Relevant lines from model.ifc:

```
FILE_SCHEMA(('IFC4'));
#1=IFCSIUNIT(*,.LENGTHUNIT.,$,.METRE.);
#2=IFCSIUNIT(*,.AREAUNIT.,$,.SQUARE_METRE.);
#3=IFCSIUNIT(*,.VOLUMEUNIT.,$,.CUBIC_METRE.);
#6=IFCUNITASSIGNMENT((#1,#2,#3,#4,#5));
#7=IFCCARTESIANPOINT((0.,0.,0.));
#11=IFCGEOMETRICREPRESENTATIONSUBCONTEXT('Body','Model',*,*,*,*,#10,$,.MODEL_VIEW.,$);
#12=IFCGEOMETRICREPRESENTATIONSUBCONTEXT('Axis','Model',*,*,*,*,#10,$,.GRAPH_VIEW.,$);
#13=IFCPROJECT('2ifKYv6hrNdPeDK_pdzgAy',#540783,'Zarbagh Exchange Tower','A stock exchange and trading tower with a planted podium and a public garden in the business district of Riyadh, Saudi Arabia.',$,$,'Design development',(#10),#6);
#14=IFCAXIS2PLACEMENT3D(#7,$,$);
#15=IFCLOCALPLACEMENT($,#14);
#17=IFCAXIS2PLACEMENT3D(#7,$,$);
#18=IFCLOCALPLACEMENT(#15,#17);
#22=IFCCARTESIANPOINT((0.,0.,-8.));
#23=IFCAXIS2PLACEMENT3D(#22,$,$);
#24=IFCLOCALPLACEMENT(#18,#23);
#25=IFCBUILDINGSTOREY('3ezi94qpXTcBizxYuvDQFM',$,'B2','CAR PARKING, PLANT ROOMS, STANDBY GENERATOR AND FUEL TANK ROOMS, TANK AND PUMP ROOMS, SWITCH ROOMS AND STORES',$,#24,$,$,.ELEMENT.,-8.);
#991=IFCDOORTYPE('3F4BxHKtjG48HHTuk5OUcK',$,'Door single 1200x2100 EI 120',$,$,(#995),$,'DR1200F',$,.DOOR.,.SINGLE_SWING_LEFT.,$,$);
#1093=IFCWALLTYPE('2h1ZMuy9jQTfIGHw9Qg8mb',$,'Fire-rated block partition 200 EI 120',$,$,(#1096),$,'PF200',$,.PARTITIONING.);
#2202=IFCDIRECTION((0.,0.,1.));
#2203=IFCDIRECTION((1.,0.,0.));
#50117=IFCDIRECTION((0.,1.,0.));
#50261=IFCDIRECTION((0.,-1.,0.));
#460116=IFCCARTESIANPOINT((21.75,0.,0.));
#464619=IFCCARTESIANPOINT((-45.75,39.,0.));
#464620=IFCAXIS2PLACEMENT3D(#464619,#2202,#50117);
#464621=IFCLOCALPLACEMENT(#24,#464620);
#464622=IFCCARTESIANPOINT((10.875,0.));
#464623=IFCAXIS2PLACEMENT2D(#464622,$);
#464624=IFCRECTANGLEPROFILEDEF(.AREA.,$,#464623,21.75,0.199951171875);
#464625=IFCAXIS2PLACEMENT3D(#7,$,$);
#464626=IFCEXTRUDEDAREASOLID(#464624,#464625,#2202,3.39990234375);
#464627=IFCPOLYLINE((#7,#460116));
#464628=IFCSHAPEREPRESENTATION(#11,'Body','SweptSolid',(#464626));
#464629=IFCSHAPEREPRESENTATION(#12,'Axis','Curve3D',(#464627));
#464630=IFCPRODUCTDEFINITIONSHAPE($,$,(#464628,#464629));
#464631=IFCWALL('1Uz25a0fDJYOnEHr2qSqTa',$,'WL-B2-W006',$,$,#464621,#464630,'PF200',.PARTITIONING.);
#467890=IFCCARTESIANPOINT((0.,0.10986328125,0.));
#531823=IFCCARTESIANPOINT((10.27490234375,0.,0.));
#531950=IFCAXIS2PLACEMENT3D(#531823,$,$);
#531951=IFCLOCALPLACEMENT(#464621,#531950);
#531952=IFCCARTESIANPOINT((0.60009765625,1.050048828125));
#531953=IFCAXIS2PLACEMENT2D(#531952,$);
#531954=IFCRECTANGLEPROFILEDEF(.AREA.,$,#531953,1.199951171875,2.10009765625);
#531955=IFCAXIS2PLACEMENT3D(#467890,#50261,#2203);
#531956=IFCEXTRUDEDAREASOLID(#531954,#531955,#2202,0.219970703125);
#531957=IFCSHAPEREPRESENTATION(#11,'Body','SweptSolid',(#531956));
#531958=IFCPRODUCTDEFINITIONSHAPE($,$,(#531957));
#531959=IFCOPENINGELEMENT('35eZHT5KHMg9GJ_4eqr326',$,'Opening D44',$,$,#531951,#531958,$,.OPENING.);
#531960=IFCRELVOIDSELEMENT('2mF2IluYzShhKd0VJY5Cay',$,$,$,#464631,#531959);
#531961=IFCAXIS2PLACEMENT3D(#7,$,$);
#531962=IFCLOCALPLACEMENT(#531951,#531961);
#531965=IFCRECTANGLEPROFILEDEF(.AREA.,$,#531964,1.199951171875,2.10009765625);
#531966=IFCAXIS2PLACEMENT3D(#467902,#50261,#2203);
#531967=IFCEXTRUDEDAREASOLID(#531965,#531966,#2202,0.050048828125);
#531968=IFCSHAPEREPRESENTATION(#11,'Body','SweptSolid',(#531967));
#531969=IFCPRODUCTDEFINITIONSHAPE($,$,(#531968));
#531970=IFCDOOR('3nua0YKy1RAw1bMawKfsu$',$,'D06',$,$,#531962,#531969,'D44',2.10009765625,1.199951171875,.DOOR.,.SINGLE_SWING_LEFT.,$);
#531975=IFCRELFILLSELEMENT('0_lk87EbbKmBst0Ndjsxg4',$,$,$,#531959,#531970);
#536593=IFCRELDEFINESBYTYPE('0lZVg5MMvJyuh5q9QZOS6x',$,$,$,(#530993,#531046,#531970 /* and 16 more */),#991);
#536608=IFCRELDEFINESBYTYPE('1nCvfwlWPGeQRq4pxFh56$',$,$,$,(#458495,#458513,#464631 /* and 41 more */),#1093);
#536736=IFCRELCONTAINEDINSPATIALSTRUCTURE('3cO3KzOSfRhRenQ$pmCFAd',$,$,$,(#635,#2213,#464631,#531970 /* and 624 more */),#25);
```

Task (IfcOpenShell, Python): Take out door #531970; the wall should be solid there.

```python
import ifcopenshell
import ifcopenshell.api.feature
import ifcopenshell.api.root
import ifcopenshell.geom
import ifcopenshell.util.shape

model = ifcopenshell.open("model.ifc")
settings = ifcopenshell.geom.settings()


def volume(element):
    """Net volume in cubic metres, openings subtracted."""
    shape = ifcopenshell.geom.create_shape(settings, element)
    return ifcopenshell.util.shape.get_volume(shape.geometry)


door = model.by_guid("3nua0YKy1RAw1bMawKfsu$")
opening = door.FillsVoids[0].RelatingOpeningElement
wall = opening.VoidsElements[0].RelatingBuildingElement
before = volume(wall)

ifcopenshell.api.root.remove_product(model, product=door)
ifcopenshell.api.feature.remove_feature(model, feature=opening)

after = volume(wall)

print(f"wall volume {before:.3f} -> {after:.3f} m3")

model.write("model_updated.ifc")
```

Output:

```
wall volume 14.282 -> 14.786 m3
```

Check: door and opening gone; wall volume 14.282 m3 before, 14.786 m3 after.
